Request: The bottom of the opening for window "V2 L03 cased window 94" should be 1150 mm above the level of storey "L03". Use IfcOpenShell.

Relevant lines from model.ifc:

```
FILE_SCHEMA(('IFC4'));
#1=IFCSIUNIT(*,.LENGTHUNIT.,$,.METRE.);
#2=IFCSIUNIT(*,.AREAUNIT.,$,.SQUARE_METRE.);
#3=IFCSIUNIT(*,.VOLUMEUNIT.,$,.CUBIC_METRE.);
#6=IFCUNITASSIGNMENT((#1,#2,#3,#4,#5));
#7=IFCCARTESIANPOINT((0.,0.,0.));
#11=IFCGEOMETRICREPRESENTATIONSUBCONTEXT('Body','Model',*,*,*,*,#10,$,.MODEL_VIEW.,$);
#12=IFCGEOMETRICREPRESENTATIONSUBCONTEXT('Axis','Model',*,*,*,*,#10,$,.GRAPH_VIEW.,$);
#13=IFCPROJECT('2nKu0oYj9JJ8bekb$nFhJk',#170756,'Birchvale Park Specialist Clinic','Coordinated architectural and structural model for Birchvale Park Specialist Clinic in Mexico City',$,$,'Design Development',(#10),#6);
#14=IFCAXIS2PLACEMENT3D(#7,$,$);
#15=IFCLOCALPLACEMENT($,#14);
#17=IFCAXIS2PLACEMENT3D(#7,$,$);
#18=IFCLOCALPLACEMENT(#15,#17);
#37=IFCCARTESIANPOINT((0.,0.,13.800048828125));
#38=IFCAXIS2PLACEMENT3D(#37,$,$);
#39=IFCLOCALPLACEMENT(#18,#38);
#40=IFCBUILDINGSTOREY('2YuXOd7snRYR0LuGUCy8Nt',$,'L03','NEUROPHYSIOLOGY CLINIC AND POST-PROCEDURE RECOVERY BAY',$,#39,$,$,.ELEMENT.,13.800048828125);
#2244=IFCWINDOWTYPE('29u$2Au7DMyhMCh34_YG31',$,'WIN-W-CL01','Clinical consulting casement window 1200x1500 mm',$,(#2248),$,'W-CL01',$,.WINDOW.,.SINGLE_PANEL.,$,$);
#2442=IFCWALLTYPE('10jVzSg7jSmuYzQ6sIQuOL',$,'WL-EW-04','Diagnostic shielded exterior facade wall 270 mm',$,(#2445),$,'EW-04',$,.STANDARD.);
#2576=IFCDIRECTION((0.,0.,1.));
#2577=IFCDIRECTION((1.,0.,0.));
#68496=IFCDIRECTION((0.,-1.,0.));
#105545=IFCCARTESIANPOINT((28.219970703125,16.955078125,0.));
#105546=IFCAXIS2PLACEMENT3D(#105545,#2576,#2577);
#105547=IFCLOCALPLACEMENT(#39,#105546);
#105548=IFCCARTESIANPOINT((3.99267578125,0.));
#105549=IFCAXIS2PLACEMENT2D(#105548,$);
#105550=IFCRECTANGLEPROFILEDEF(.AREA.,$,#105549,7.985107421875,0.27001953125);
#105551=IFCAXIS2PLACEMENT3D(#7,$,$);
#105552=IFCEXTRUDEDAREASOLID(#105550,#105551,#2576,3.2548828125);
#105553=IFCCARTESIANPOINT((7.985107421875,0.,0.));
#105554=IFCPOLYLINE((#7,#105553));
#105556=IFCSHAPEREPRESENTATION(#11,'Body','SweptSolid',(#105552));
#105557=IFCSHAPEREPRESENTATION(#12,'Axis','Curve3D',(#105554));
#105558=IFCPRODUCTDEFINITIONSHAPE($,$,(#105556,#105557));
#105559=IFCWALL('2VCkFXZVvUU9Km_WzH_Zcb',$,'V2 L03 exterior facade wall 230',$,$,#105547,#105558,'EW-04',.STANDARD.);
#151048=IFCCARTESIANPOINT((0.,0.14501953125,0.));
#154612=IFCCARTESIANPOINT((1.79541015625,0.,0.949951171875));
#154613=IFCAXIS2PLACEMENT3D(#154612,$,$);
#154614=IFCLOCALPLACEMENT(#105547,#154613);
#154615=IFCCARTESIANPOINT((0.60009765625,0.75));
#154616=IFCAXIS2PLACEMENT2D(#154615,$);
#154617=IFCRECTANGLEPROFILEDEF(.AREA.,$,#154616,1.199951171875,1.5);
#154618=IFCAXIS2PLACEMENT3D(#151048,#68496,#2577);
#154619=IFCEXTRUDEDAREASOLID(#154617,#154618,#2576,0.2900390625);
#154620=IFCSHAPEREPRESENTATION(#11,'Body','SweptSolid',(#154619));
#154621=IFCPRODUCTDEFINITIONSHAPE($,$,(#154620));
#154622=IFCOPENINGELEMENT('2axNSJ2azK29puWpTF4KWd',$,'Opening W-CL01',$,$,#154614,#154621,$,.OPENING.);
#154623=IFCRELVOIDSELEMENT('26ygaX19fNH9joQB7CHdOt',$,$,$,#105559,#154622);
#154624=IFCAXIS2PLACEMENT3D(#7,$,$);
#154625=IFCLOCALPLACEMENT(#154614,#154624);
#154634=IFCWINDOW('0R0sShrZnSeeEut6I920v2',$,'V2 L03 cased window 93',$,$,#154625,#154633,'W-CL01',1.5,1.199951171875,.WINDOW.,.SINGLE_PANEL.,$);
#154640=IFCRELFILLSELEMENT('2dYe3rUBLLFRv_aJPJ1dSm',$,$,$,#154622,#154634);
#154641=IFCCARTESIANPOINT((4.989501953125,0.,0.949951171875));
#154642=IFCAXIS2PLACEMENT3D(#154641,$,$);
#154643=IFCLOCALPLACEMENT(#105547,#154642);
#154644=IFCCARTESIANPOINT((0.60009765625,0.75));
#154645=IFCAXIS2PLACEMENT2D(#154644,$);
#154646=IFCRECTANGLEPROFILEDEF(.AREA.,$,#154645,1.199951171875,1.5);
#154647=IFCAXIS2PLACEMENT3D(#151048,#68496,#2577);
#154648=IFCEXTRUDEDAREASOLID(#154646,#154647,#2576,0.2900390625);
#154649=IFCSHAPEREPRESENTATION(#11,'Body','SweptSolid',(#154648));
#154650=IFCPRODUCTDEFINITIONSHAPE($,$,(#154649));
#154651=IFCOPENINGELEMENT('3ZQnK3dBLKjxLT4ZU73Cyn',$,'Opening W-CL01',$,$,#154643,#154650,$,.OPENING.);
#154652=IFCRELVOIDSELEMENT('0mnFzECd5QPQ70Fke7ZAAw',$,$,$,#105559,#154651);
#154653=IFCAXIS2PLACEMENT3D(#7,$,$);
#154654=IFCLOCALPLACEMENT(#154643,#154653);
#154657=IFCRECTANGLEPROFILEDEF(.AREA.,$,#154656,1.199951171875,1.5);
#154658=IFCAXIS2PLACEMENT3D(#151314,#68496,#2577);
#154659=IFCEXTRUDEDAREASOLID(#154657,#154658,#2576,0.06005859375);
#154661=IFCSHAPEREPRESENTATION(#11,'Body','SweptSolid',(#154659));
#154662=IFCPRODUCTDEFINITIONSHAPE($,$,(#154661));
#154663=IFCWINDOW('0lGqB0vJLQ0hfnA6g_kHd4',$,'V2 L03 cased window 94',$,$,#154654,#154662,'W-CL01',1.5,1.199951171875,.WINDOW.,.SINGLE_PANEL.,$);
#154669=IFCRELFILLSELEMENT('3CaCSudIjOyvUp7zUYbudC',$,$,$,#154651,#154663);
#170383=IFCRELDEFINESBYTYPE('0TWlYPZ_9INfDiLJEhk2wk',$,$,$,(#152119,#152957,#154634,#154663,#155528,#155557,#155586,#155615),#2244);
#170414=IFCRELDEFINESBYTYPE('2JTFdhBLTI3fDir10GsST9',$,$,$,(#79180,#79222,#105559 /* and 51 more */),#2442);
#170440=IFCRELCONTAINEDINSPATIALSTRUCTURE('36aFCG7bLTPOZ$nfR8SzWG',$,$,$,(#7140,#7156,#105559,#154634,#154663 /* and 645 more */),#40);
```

```python
import numpy as np
import ifcopenshell
import ifcopenshell.api.geometry
import ifcopenshell.geom
import ifcopenshell.util.element
import ifcopenshell.util.placement
import ifcopenshell.util.shape
import ifcopenshell.util.unit

model = ifcopenshell.open("model.ifc")
unit_scale = ifcopenshell.util.unit.calculate_unit_scale(model)

window = model.by_guid("0lGqB0vJLQ0hfnA6g_kHd4")
opening = window.FillsVoids[0].RelatingOpeningElement
storey = ifcopenshell.util.element.get_container(window, ifc_class="IfcBuildingStorey")
level = ifcopenshell.util.placement.get_local_placement(storey.ObjectPlacement)[2, 3]

# The opening's origin need not be at the sill, so measure its lowest point.
shape = ifcopenshell.geom.create_shape(ifcopenshell.geom.settings(), opening)
bottom = ifcopenshell.util.shape.get_shape_bottom_elevation(shape, shape.geometry) / unit_scale
dz = level + 1.15 - bottom

shift = np.array([0.0, 0.0, dz])
# The window is placed relative to its opening, so it follows when the opening moves.
matrix = ifcopenshell.util.placement.get_local_placement(opening.ObjectPlacement)
matrix[:3, 3] += shift
ifcopenshell.api.geometry.edit_object_placement(
    model, product=opening, matrix=matrix, is_si=False, should_transform_children=True
)

print(f"moved by {dz * unit_scale:+.3f} m")

model.write("model_rev.ifc")
```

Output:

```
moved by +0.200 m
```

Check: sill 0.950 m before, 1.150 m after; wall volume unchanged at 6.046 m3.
